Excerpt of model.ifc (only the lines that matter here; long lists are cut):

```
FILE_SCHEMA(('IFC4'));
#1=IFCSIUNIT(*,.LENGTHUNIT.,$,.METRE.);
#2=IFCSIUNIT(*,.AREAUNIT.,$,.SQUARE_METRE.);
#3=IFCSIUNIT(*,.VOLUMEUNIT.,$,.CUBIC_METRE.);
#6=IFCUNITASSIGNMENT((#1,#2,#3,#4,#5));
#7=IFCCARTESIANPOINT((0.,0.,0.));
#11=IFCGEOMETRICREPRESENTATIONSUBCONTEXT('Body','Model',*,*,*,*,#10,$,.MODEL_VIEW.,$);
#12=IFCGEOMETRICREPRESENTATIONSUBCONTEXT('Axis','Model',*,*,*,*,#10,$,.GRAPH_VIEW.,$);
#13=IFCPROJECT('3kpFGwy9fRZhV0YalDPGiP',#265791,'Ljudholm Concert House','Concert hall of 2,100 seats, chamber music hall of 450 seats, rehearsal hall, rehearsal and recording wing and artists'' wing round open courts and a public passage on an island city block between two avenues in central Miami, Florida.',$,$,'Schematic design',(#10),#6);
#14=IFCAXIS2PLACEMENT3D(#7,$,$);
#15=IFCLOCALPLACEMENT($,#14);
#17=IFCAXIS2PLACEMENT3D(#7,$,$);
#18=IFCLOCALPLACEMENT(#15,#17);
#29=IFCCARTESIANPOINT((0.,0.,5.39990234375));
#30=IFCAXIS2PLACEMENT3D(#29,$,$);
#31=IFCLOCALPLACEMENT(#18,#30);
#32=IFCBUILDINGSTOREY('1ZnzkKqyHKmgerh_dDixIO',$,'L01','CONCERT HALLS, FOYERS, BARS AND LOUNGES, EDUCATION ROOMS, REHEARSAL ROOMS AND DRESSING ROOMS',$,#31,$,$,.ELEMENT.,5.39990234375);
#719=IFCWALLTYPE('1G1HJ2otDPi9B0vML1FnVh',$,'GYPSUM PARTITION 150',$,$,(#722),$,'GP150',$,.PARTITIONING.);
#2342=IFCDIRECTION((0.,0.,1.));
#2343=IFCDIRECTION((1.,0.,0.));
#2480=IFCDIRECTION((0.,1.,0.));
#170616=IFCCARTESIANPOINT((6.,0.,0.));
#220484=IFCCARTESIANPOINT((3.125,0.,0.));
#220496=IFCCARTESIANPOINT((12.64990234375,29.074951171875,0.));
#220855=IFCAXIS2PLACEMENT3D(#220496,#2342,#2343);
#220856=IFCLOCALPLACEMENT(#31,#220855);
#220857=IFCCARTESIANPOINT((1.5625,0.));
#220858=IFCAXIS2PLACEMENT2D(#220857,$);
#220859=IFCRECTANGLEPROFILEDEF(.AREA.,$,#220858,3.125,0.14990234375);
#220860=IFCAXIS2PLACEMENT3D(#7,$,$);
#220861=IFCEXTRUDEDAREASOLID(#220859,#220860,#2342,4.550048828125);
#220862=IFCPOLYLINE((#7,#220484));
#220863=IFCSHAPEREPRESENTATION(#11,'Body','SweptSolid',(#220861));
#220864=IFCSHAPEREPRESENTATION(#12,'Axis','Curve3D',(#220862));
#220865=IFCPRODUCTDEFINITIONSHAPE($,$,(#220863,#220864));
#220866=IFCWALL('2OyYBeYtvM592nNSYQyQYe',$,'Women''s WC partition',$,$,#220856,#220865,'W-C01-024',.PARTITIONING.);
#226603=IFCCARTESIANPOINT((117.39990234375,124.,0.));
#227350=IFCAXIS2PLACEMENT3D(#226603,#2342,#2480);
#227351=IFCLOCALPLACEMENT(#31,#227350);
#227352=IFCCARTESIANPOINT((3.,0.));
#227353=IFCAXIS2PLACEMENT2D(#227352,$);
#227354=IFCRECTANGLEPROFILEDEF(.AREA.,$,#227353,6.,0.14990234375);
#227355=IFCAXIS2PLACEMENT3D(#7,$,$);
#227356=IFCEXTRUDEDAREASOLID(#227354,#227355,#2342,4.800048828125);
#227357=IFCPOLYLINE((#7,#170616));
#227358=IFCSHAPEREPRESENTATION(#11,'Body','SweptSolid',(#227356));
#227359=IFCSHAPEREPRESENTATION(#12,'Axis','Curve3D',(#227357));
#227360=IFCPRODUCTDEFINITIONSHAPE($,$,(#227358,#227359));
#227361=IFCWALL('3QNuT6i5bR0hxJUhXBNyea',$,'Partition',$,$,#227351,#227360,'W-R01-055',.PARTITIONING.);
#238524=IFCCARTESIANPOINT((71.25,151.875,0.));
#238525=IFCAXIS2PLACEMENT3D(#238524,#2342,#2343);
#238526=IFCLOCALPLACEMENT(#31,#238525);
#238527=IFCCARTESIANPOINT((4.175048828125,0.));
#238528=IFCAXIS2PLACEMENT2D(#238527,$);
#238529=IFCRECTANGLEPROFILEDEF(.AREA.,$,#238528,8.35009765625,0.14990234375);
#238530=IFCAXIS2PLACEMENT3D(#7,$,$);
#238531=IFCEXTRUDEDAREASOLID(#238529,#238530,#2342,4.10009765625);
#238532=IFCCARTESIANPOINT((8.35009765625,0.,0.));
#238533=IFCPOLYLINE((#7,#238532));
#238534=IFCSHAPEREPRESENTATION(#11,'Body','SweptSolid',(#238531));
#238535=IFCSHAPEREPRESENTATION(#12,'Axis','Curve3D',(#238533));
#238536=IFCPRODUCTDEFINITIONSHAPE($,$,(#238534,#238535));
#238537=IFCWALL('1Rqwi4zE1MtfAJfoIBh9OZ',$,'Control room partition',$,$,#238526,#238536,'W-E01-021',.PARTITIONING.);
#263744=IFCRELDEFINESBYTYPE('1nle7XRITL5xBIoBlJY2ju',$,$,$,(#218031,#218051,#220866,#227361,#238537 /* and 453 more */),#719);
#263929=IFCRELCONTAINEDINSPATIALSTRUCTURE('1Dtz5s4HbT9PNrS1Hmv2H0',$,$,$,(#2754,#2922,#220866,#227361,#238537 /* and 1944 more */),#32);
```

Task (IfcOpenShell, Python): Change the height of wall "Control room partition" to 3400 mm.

```python
import ifcopenshell
import ifcopenshell.geom
import ifcopenshell.util.representation
import ifcopenshell.util.shape
import ifcopenshell.util.unit

model = ifcopenshell.open("model.ifc")
unit_scale = ifcopenshell.util.unit.calculate_unit_scale(model)
settings = ifcopenshell.geom.settings()


def volume(element):
    """Net volume in cubic metres, openings subtracted."""
    shape = ifcopenshell.geom.create_shape(settings, element)
    return ifcopenshell.util.shape.get_volume(shape.geometry)


wall = model.by_guid("1Rqwi4zE1MtfAJfoIBh9OZ")
before = volume(wall)

body = ifcopenshell.util.representation.get_representation(wall, "Model", "Body")
solid = body.Items[0]
old_height = solid.Depth
solid.Depth = 3.4 / unit_scale
after = volume(wall)

print(f"height {old_height:g} -> {solid.Depth:g}, volume {before:.3f} -> {after:.3f} m3")

model.write("model_updated.ifc")
```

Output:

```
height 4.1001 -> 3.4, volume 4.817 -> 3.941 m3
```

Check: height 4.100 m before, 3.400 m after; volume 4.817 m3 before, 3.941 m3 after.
